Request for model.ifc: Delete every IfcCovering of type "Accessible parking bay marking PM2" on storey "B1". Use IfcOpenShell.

First a look at what the model holds.

```python
import ifcopenshell
import ifcopenshell.util.element

model = ifcopenshell.open("model.ifc")
print(model.schema)
storey = next(s for s in model.by_type("IfcBuildingStorey") if s.Name == "B1")
coverings = [e for e in ifcopenshell.util.element.get_decomposition(storey) if e.is_a("IfcCovering")]
seen = {}
for e in coverings:
    element_type = ifcopenshell.util.element.get_type(e)
    name = element_type.Name if element_type not in (None, e) else None
    seen[name] = seen.get(name, 0) + 1
for name, count in sorted(seen.items(), key=str):
    print(count, "x", name)
```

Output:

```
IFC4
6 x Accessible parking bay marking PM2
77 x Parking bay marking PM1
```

```python
import ifcopenshell
import ifcopenshell.api.root
import ifcopenshell.util.element

model = ifcopenshell.open("model.ifc")

storey = next(s for s in model.by_type("IfcBuildingStorey") if s.Name == "B1")
coverings = [e for e in ifcopenshell.util.element.get_decomposition(storey) if e.is_a("IfcCovering")]
targets = [e for e in coverings if (t := ifcopenshell.util.element.get_type(e)) not in (None, e) and t.Name == "Accessible parking bay marking PM2"]

for e in targets:
    ifcopenshell.api.root.remove_product(model, product=e)
print(len(targets), "removed")

model.write("model_v2.ifc")
```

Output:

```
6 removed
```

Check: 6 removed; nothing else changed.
